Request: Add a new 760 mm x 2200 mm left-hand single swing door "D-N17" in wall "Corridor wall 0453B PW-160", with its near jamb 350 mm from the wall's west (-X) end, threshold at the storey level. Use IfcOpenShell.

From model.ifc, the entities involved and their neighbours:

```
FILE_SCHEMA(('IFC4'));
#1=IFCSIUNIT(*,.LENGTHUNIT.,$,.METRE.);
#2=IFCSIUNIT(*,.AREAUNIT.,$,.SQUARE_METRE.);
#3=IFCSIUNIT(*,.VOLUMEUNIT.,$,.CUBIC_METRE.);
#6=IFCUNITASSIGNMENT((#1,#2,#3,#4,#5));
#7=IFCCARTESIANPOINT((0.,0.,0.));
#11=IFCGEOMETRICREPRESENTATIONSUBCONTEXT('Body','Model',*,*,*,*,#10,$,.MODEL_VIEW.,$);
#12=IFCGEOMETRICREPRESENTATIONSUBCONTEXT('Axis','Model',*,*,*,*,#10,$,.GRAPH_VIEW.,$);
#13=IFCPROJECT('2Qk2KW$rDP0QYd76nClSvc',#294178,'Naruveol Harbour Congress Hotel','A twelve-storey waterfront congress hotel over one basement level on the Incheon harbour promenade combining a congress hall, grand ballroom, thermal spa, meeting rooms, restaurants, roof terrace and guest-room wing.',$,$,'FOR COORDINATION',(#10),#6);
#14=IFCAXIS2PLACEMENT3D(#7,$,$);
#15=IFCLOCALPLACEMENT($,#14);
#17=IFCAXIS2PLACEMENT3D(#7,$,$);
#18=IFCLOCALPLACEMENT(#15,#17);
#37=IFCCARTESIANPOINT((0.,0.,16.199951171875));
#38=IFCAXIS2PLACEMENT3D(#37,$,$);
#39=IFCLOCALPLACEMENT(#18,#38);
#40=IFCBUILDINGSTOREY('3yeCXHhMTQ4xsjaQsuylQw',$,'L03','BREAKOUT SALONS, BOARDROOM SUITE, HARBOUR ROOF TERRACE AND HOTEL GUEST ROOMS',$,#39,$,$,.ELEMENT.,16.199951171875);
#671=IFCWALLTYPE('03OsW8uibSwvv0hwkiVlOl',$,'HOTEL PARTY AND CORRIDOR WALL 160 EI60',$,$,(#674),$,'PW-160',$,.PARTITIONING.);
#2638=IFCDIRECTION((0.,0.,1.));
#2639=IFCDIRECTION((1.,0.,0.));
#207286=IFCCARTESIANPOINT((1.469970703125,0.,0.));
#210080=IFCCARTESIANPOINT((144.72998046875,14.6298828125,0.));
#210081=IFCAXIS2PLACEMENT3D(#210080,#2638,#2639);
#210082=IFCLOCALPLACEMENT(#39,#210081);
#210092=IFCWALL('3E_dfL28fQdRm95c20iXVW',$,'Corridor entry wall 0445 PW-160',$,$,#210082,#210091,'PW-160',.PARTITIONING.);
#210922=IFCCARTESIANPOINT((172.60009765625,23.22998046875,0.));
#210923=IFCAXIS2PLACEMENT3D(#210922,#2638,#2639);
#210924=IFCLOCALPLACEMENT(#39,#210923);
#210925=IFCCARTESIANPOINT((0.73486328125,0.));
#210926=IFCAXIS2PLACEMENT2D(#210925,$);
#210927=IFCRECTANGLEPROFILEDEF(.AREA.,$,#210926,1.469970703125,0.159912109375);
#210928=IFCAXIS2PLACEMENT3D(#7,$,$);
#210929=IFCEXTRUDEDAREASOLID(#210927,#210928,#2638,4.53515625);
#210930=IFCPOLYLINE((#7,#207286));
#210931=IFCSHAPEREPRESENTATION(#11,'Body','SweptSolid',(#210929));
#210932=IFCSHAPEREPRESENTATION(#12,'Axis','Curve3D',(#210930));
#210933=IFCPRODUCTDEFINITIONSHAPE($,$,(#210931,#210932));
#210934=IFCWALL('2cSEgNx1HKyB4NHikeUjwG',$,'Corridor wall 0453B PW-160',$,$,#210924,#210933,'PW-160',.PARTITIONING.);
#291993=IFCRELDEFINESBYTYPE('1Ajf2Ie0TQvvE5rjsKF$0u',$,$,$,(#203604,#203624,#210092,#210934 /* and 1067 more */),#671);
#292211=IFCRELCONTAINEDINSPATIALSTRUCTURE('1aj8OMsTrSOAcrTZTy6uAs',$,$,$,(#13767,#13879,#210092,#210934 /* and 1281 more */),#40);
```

```python
import numpy as np
import ifcopenshell
import ifcopenshell.api.feature
import ifcopenshell.api.geometry
import ifcopenshell.api.root
import ifcopenshell.api.spatial
import ifcopenshell.geom
import ifcopenshell.util.element
import ifcopenshell.util.placement
import ifcopenshell.util.representation
import ifcopenshell.util.shape
import ifcopenshell.util.unit

model = ifcopenshell.open("model.ifc")
unit_scale = ifcopenshell.util.unit.calculate_unit_scale(model)
settings = ifcopenshell.geom.settings()


def volume(element):
    """Net volume in cubic metres, openings subtracted."""
    shape = ifcopenshell.geom.create_shape(settings, element)
    return ifcopenshell.util.shape.get_volume(shape.geometry)


wall = model.by_guid("2cSEgNx1HKyB4NHikeUjwG")
storey = ifcopenshell.util.element.get_container(wall, ifc_class="IfcBuildingStorey")
context = ifcopenshell.util.representation.get_context(model, "Model", "Body", "MODEL_VIEW")
before = volume(wall)

width, height, from_end, sill = 0.76, 2.2, 0.35, 0.0  # metres

# The wall runs along its own X axis, and the end named is its -X end.
wall_shape = ifcopenshell.geom.create_shape(settings, wall)
x, y, z = ifcopenshell.util.shape.get_vertices(wall_shape.geometry).T
start = x.min() + from_end
face, thickness = float(y.min()), float(y.max() - y.min())
wall_matrix = ifcopenshell.util.placement.get_local_placement(wall.ObjectPlacement)
level = ifcopenshell.util.placement.get_local_placement(storey.ObjectPlacement)[2, 3]


def in_wall(x, y):
    """Placement at x, y metres in the wall's axes, at sill height."""
    matrix = wall_matrix.copy()
    matrix[:, 3] = wall_matrix @ np.array([x / unit_scale, y / unit_scale, 0.0, 1.0])
    matrix[2, 3] = level + sill / unit_scale
    return matrix


# Opening: a box that overshoots both wall faces by 50 mm.
opening = ifcopenshell.api.root.create_entity(model, ifc_class="IfcOpeningElement", predefined_type="OPENING")
box = ifcopenshell.api.geometry.add_wall_representation(
    model, context=context, length=width, height=height, thickness=thickness + 0.1
)
ifcopenshell.api.geometry.assign_representation(model, product=opening, representation=box)
ifcopenshell.api.geometry.edit_object_placement(model, product=opening, matrix=in_wall(start, face - 0.05), is_si=False)
ifcopenshell.api.feature.add_feature(model, feature=opening, element=wall)

door = ifcopenshell.api.root.create_entity(model, ifc_class="IfcDoor", name="D-N17", predefined_type="DOOR")
door.OverallWidth, door.OverallHeight = width / unit_scale, height / unit_scale
door.OperationType = "SINGLE_SWING_LEFT"
body = ifcopenshell.api.geometry.add_door_representation(
    model,
    context=context,
    overall_width=door.OverallWidth,
    overall_height=door.OverallHeight,
    operation_type="SINGLE_SWING_LEFT",
    lining_properties={"LiningDepth": thickness / unit_scale, "ThresholdDepth": thickness / unit_scale},
)
ifcopenshell.api.geometry.assign_representation(model, product=door, representation=body)
ifcopenshell.api.spatial.assign_container(model, products=[door], relating_structure=storey)
ifcopenshell.api.feature.add_filling(model, opening=opening, element=door)

# The lining spans the wall, so the door starts at the wall face.
ifcopenshell.api.geometry.edit_object_placement(model, product=door, matrix=in_wall(start, face), is_si=False)

after = volume(wall)

print(f"wall volume {before:.3f} -> {after:.3f} m3")

model.write("model_rev.ifc")
```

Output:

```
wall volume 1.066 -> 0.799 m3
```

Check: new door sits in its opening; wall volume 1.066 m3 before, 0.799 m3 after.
